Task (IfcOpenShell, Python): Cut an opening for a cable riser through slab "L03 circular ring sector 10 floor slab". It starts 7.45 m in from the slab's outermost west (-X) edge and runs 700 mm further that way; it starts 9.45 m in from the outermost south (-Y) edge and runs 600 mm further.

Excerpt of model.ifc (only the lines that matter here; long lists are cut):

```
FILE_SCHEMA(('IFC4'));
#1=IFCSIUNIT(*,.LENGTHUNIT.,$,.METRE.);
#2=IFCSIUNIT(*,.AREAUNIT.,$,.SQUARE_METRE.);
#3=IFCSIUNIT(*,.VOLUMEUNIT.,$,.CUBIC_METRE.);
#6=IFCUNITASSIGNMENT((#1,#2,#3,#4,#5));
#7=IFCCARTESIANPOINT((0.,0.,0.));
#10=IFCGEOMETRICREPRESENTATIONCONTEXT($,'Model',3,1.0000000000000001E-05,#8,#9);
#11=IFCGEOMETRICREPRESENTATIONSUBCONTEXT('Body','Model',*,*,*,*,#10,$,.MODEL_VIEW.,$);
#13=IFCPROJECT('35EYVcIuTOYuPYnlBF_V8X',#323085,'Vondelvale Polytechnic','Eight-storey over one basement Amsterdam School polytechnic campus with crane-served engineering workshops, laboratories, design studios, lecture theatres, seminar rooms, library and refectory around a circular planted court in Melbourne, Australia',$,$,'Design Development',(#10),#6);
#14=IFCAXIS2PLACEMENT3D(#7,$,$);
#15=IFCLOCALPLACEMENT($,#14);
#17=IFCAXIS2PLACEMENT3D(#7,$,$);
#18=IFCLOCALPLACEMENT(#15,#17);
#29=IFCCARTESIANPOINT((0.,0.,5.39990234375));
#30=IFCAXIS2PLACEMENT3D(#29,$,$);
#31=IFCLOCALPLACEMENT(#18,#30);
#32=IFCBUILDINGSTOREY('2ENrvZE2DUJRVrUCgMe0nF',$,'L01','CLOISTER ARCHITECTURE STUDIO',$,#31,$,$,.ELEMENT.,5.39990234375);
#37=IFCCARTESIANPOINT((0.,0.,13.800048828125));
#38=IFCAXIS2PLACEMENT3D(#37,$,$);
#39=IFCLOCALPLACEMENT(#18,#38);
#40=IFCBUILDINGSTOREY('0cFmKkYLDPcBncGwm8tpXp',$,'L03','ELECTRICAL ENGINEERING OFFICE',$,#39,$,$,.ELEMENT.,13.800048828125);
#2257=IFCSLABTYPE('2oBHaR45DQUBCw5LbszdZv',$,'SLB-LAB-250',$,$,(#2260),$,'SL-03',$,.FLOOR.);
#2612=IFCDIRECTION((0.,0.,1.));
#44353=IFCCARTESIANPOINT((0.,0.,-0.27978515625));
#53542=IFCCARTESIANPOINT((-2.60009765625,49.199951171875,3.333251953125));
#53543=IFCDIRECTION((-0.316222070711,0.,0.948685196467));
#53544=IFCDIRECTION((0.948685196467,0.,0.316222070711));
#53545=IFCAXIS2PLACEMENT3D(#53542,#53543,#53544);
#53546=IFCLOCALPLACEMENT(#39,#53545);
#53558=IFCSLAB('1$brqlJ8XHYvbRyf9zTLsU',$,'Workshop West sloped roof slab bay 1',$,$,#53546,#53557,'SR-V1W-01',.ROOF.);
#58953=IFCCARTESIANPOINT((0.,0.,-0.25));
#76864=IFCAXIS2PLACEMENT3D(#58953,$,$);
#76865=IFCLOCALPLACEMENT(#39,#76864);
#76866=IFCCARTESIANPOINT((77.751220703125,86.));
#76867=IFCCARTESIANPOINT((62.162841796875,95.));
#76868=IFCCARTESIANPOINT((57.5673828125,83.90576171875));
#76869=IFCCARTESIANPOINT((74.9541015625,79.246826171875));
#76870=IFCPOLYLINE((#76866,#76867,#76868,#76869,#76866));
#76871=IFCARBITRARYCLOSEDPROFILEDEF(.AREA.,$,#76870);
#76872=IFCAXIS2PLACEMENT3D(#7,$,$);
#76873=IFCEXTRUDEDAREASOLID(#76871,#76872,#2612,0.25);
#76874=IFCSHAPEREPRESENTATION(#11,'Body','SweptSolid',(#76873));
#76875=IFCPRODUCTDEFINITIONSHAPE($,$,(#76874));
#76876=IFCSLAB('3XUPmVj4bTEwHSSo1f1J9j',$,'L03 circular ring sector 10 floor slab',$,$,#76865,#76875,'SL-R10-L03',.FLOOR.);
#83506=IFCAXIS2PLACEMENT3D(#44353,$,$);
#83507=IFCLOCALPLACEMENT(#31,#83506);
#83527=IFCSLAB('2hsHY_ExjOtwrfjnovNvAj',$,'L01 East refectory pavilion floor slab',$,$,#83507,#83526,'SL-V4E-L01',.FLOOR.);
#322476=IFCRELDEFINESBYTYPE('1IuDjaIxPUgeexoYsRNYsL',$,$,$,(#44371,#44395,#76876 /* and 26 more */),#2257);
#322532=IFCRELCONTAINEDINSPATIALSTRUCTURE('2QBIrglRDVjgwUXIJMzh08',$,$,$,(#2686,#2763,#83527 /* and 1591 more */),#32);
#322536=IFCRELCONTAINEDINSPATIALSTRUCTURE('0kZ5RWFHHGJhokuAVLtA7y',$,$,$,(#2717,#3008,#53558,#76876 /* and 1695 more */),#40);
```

```python
import numpy as np
import ifcopenshell
import ifcopenshell.api.feature
import ifcopenshell.api.geometry
import ifcopenshell.api.root
import ifcopenshell.geom
import ifcopenshell.util.placement
import ifcopenshell.util.representation
import ifcopenshell.util.shape
import ifcopenshell.util.unit

model = ifcopenshell.open("model.ifc")
unit_scale = ifcopenshell.util.unit.calculate_unit_scale(model)
settings = ifcopenshell.geom.settings()


def volume(element):
    """Net volume in cubic metres, openings subtracted."""
    shape = ifcopenshell.geom.create_shape(settings, element)
    return ifcopenshell.util.shape.get_volume(shape.geometry)


slab = model.by_guid("3XUPmVj4bTEwHSSo1f1J9j")
before = volume(slab)

# Extent in the slab's own axes, in metres. The edges named are its -X and -Y sides.
slab_shape = ifcopenshell.geom.create_shape(settings, slab)
vertices = ifcopenshell.util.shape.get_vertices(slab_shape.geometry)
x_min, y_min, bottom = vertices.min(axis=0)
top = vertices[:, 2].max()

opening = ifcopenshell.api.root.create_entity(model, ifc_class="IfcOpeningElement", name="Cable riser opening", predefined_type="OPENING")
context = ifcopenshell.util.representation.get_context(model, "Model", "Body", "MODEL_VIEW")
width, depth = 0.7, 0.6
outline = [(0.0, 0.0), (width, 0.0), (width, depth), (0.0, depth), (0.0, 0.0)]
# Overshoot both faces by 50 mm so the cut is clean.
shape = ifcopenshell.api.geometry.add_slab_representation(
    model, context=context, depth=top - bottom + 0.1, polyline=outline
)
ifcopenshell.api.geometry.assign_representation(model, product=opening, representation=shape)

matrix = ifcopenshell.util.placement.get_local_placement(slab.ObjectPlacement)
matrix[:, 3] = matrix @ np.append(np.array([x_min + 7.45, y_min + 9.45, bottom - 0.05]) / unit_scale, 1.0)
ifcopenshell.api.geometry.edit_object_placement(model, product=opening, matrix=matrix, is_si=False)
ifcopenshell.api.feature.add_feature(model, feature=opening, element=slab)

after = volume(slab)

print(f"slab volume {before:.3f} -> {after:.3f} m3")

model.write("model-out.ifc")
```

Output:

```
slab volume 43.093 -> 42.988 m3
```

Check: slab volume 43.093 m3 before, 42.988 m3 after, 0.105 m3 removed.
